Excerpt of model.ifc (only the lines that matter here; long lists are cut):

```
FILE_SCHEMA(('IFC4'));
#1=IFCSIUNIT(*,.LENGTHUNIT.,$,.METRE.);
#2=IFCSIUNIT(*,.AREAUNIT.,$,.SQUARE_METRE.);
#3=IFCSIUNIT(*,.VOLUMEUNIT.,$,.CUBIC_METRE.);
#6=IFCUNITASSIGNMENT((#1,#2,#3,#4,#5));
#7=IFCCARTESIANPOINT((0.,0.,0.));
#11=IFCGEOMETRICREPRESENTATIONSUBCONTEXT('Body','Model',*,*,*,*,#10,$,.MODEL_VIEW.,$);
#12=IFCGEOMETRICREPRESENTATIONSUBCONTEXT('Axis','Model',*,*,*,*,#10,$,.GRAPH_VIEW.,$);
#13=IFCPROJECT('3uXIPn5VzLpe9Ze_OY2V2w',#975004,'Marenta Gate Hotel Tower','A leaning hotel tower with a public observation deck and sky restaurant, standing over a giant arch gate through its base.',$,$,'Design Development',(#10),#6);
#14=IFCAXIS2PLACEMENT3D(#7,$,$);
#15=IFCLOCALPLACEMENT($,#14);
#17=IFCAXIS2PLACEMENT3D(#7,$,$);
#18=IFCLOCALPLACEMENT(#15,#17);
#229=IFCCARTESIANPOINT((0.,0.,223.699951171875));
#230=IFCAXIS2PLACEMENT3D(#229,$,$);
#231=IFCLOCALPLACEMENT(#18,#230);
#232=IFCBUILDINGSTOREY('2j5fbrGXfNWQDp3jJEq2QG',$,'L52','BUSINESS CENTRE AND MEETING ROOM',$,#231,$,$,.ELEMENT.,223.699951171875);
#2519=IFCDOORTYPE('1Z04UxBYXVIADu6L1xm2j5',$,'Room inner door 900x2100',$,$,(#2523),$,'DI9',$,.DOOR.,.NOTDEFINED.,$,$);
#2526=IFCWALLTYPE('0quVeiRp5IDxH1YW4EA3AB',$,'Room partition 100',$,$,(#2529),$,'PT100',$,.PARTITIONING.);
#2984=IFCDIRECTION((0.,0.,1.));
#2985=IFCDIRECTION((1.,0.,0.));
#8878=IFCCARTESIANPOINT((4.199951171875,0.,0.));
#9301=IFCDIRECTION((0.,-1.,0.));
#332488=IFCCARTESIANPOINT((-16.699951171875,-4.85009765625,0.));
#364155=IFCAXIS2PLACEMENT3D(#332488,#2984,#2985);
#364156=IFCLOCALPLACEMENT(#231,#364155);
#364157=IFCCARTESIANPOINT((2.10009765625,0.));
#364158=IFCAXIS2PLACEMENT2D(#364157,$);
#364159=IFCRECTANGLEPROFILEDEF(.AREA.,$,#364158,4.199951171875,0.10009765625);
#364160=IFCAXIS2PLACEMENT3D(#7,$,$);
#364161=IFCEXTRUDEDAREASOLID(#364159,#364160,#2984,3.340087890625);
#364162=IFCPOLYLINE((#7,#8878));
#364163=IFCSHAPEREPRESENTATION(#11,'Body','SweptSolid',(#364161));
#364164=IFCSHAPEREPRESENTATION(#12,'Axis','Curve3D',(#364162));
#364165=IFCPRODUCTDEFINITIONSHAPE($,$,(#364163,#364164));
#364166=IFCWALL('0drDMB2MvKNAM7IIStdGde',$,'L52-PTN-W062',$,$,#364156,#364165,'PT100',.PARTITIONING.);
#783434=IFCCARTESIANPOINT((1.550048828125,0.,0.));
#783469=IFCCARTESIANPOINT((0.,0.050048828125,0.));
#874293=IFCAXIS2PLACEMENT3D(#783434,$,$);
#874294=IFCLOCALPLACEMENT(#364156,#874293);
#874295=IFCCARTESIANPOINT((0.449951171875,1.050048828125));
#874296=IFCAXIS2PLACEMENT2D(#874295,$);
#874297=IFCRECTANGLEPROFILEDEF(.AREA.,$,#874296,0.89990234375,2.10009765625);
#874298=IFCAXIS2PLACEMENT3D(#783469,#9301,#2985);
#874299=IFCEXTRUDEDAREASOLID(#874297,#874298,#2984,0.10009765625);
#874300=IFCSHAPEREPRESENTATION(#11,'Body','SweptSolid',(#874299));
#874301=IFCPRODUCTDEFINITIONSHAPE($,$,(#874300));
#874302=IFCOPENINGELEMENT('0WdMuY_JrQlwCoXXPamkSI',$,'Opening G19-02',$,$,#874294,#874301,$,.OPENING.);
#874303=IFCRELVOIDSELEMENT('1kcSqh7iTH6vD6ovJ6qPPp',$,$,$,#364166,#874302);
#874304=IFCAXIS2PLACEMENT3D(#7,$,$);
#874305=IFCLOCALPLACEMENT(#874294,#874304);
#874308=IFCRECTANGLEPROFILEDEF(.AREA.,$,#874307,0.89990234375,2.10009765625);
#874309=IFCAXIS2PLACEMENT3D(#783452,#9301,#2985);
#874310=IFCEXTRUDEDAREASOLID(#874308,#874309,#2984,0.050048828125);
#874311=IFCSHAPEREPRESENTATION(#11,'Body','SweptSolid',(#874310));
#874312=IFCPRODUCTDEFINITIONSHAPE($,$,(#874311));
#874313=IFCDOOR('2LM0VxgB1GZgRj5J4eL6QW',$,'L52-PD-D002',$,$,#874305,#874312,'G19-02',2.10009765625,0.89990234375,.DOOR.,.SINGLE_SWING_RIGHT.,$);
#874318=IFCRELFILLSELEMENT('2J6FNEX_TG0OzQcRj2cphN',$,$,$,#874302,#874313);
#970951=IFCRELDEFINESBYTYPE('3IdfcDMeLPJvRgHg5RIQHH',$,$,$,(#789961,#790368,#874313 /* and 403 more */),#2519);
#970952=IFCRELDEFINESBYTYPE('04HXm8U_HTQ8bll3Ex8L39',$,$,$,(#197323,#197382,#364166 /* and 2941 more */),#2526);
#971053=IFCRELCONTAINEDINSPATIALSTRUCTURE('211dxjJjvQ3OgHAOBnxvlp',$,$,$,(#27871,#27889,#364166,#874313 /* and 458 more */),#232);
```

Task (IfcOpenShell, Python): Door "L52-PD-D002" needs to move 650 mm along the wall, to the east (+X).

```python
import ifcopenshell
import ifcopenshell.api.geometry
import ifcopenshell.util.placement
import ifcopenshell.util.unit

model = ifcopenshell.open("model.ifc")
unit_scale = ifcopenshell.util.unit.calculate_unit_scale(model)

door = model.by_guid("2LM0VxgB1GZgRj5J4eL6QW")
opening = door.FillsVoids[0].RelatingOpeningElement
wall = opening.VoidsElements[0].RelatingBuildingElement

wall_matrix = ifcopenshell.util.placement.get_local_placement(wall.ObjectPlacement)
shift = wall_matrix[:3, 0] * 0.65 / unit_scale
before = ifcopenshell.util.placement.get_local_placement(door.ObjectPlacement)[:3, 3].copy()

# The door is placed relative to its opening, so it follows when the opening moves.
matrix = ifcopenshell.util.placement.get_local_placement(opening.ObjectPlacement)
matrix[:3, 3] += shift
ifcopenshell.api.geometry.edit_object_placement(
    model, product=opening, matrix=matrix, is_si=False, should_transform_children=True
)

after = ifcopenshell.util.placement.get_local_placement(door.ObjectPlacement)[:3, 3]
print("door moved by", (after - before).round(3) + 0.0)

model.write("model_edited.ifc")
```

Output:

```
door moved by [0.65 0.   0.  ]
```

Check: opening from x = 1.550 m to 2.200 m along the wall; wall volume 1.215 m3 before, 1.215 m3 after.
